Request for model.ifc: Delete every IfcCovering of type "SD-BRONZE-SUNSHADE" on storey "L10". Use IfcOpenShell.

First a look at what the model holds.

```python
import ifcopenshell
import ifcopenshell.util.element

model = ifcopenshell.open("model.ifc")
print(model.schema)
storey = next(s for s in model.by_type("IfcBuildingStorey") if s.Name == "L10")
coverings = [e for e in ifcopenshell.util.element.get_decomposition(storey) if e.is_a("IfcCovering")]
seen = {}
for e in coverings:
    element_type = ifcopenshell.util.element.get_type(e)
    name = element_type.Name if element_type not in (None, e) else None
    seen[name] = seen.get(name, 0) + 1
for name, count in sorted(seen.items(), key=str):
    print(count, "x", name)
```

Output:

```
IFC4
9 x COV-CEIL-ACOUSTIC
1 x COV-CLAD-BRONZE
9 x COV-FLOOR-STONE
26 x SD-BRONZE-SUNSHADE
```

```python
import ifcopenshell
import ifcopenshell.api.root
import ifcopenshell.util.element

model = ifcopenshell.open("model.ifc")

storey = next(s for s in model.by_type("IfcBuildingStorey") if s.Name == "L10")
coverings = [e for e in ifcopenshell.util.element.get_decomposition(storey) if e.is_a("IfcCovering")]
targets = [e for e in coverings if (t := ifcopenshell.util.element.get_type(e)) not in (None, e) and t.Name == "SD-BRONZE-SUNSHADE"]

for e in targets:
    ifcopenshell.api.root.remove_product(model, product=e)
print(len(targets), "removed")

model.write("model_v2.ifc")
```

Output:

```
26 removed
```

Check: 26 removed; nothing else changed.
